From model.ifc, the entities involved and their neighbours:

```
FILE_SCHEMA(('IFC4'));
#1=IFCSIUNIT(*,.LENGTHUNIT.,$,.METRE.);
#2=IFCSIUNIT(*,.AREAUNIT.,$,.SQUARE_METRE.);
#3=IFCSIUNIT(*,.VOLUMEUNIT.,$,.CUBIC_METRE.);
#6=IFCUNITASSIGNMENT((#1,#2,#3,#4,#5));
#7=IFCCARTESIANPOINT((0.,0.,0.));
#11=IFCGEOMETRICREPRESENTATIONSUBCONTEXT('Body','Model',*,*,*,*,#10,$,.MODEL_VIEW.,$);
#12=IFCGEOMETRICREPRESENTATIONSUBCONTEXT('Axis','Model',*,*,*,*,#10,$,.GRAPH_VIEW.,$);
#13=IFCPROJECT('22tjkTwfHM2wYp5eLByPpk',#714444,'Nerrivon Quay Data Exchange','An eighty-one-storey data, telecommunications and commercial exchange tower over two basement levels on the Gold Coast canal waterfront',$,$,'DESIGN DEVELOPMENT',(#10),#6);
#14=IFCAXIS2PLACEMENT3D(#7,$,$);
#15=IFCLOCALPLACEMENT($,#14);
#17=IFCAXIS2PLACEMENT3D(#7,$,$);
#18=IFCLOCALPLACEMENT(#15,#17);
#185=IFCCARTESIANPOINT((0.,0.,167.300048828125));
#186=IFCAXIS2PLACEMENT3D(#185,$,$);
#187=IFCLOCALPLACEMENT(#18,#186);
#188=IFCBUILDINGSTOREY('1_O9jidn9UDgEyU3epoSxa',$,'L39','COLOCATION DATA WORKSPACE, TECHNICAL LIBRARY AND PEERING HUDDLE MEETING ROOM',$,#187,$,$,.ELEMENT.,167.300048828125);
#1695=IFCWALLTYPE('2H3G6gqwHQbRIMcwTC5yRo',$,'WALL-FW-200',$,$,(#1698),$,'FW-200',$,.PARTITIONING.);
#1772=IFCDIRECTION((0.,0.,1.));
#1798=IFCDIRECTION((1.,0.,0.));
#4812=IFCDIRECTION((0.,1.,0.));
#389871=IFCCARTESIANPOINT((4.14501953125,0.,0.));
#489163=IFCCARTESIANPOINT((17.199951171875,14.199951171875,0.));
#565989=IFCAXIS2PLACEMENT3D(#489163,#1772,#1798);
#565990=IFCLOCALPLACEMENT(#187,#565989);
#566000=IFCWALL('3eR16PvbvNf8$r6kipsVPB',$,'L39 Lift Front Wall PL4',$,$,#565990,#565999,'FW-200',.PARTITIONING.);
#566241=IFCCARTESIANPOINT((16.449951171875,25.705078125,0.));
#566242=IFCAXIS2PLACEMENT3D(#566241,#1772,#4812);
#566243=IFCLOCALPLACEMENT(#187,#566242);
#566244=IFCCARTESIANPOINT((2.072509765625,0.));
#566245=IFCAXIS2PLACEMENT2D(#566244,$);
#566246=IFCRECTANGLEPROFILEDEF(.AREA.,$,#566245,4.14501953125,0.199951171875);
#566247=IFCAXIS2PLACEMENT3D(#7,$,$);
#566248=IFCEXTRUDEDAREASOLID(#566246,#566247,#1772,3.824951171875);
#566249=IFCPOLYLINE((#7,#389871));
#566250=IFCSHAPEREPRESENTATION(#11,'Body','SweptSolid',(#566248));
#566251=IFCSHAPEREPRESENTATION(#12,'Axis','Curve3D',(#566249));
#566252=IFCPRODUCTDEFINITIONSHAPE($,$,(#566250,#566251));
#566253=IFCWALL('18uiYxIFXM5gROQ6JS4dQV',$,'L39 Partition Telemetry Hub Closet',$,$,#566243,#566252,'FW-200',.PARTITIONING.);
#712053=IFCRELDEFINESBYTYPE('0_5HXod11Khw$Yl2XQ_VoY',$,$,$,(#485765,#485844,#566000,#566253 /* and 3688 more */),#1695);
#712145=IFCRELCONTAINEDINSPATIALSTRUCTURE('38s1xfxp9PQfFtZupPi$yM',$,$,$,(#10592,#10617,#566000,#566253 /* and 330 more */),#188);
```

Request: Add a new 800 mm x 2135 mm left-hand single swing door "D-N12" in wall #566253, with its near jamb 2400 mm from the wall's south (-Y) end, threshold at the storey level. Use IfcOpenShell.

```python
import numpy as np
import ifcopenshell
import ifcopenshell.api.feature
import ifcopenshell.api.geometry
import ifcopenshell.api.root
import ifcopenshell.api.spatial
import ifcopenshell.geom
import ifcopenshell.util.element
import ifcopenshell.util.placement
import ifcopenshell.util.representation
import ifcopenshell.util.shape
import ifcopenshell.util.unit

model = ifcopenshell.open("model.ifc")
unit_scale = ifcopenshell.util.unit.calculate_unit_scale(model)
settings = ifcopenshell.geom.settings()


def volume(element):
    """Net volume in cubic metres, openings subtracted."""
    shape = ifcopenshell.geom.create_shape(settings, element)
    return ifcopenshell.util.shape.get_volume(shape.geometry)


wall = model.by_guid("18uiYxIFXM5gROQ6JS4dQV")
storey = ifcopenshell.util.element.get_container(wall, ifc_class="IfcBuildingStorey")
context = ifcopenshell.util.representation.get_context(model, "Model", "Body", "MODEL_VIEW")
before = volume(wall)

width, height, from_end, sill = 0.8, 2.135, 2.4, 0.0  # metres

# The wall runs along its own X axis, and the end named is its -X end.
wall_shape = ifcopenshell.geom.create_shape(settings, wall)
x, y, z = ifcopenshell.util.shape.get_vertices(wall_shape.geometry).T
start = x.min() + from_end
face, thickness = float(y.min()), float(y.max() - y.min())
wall_matrix = ifcopenshell.util.placement.get_local_placement(wall.ObjectPlacement)
level = ifcopenshell.util.placement.get_local_placement(storey.ObjectPlacement)[2, 3]


def in_wall(x, y):
    """Placement at x, y metres in the wall's axes, at sill height."""
    matrix = wall_matrix.copy()
    matrix[:, 3] = wall_matrix @ np.array([x / unit_scale, y / unit_scale, 0.0, 1.0])
    matrix[2, 3] = level + sill / unit_scale
    return matrix


# Opening: a box that overshoots both wall faces by 50 mm.
opening = ifcopenshell.api.root.create_entity(model, ifc_class="IfcOpeningElement", predefined_type="OPENING")
box = ifcopenshell.api.geometry.add_wall_representation(
    model, context=context, length=width, height=height, thickness=thickness + 0.1
)
ifcopenshell.api.geometry.assign_representation(model, product=opening, representation=box)
ifcopenshell.api.geometry.edit_object_placement(model, product=opening, matrix=in_wall(start, face - 0.05), is_si=False)
ifcopenshell.api.feature.add_feature(model, feature=opening, element=wall)

door = ifcopenshell.api.root.create_entity(model, ifc_class="IfcDoor", name="D-N12", predefined_type="DOOR")
door.OverallWidth, door.OverallHeight = width / unit_scale, height / unit_scale
door.OperationType = "SINGLE_SWING_LEFT"
body = ifcopenshell.api.geometry.add_door_representation(
    model,
    context=context,
    overall_width=door.OverallWidth,
    overall_height=door.OverallHeight,
    operation_type="SINGLE_SWING_LEFT",
    lining_properties={"LiningDepth": thickness / unit_scale, "ThresholdDepth": thickness / unit_scale},
)
ifcopenshell.api.geometry.assign_representation(model, product=door, representation=body)
ifcopenshell.api.spatial.assign_container(model, products=[door], relating_structure=storey)
ifcopenshell.api.feature.add_filling(model, opening=opening, element=door)

# The lining spans the wall, so the door starts at the wall face.
ifcopenshell.api.geometry.edit_object_placement(model, product=door, matrix=in_wall(start, face), is_si=False)

after = volume(wall)

print(f"wall volume {before:.3f} -> {after:.3f} m3")

model.write("model_v2.ifc")
```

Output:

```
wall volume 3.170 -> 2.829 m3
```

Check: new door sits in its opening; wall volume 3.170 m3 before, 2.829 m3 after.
